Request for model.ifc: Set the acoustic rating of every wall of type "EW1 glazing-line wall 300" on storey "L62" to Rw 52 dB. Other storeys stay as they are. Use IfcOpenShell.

First a look at what the model holds.

```python
import ifcopenshell
import ifcopenshell.util.element

model = ifcopenshell.open("model.ifc")
print(model.schema)
storey = next(s for s in model.by_type("IfcBuildingStorey") if s.Name == "L62")
walls = [e for e in ifcopenshell.util.element.get_decomposition(storey) if e.is_a("IfcWall")]
seen = {}
for e in walls:
    element_type = ifcopenshell.util.element.get_type(e)
    key = (element_type.Name if element_type != e and element_type else None, ifcopenshell.util.element.get_pset(e, "Pset_WallCommon", "AcousticRating"))
    seen[key] = seen.get(key, 0) + 1
for (name, value), count in sorted(seen.items(), key=str):
    print(count, "x", name, "|", value)
```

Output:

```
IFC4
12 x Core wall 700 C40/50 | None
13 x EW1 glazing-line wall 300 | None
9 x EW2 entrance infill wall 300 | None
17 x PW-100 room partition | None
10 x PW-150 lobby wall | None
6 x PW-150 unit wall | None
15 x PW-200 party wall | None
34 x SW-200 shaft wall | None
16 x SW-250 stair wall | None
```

```python
import ifcopenshell
import ifcopenshell.api.pset
import ifcopenshell.util.element

model = ifcopenshell.open("model.ifc")

storey = next(s for s in model.by_type("IfcBuildingStorey") if s.Name == "L62")
walls = [e for e in ifcopenshell.util.element.get_decomposition(storey) if e.is_a("IfcWall")]

count = 0
for e in walls:
    element_type = ifcopenshell.util.element.get_type(e)
    if element_type in (None, e) or element_type.Name != "EW1 glazing-line wall 300":
        continue
    found = ifcopenshell.util.element.get_pset(e, "Pset_WallCommon", should_inherit=False)
    if found:
        pset = model.by_id(found["id"])
        if len(ifcopenshell.util.element.get_elements_by_pset(pset)) > 1:
            pset = ifcopenshell.api.pset.unshare_pset(model, products=[e], pset=pset)[0]
    else:
        pset = ifcopenshell.api.pset.add_pset(model, product=e, name="Pset_WallCommon")
    ifcopenshell.api.pset.edit_pset(model, pset=pset, properties={"AcousticRating": "Rw 52 dB"})
    count += 1

print(count, "walls updated")

model.write("model_rev.ifc")
```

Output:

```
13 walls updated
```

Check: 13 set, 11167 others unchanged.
